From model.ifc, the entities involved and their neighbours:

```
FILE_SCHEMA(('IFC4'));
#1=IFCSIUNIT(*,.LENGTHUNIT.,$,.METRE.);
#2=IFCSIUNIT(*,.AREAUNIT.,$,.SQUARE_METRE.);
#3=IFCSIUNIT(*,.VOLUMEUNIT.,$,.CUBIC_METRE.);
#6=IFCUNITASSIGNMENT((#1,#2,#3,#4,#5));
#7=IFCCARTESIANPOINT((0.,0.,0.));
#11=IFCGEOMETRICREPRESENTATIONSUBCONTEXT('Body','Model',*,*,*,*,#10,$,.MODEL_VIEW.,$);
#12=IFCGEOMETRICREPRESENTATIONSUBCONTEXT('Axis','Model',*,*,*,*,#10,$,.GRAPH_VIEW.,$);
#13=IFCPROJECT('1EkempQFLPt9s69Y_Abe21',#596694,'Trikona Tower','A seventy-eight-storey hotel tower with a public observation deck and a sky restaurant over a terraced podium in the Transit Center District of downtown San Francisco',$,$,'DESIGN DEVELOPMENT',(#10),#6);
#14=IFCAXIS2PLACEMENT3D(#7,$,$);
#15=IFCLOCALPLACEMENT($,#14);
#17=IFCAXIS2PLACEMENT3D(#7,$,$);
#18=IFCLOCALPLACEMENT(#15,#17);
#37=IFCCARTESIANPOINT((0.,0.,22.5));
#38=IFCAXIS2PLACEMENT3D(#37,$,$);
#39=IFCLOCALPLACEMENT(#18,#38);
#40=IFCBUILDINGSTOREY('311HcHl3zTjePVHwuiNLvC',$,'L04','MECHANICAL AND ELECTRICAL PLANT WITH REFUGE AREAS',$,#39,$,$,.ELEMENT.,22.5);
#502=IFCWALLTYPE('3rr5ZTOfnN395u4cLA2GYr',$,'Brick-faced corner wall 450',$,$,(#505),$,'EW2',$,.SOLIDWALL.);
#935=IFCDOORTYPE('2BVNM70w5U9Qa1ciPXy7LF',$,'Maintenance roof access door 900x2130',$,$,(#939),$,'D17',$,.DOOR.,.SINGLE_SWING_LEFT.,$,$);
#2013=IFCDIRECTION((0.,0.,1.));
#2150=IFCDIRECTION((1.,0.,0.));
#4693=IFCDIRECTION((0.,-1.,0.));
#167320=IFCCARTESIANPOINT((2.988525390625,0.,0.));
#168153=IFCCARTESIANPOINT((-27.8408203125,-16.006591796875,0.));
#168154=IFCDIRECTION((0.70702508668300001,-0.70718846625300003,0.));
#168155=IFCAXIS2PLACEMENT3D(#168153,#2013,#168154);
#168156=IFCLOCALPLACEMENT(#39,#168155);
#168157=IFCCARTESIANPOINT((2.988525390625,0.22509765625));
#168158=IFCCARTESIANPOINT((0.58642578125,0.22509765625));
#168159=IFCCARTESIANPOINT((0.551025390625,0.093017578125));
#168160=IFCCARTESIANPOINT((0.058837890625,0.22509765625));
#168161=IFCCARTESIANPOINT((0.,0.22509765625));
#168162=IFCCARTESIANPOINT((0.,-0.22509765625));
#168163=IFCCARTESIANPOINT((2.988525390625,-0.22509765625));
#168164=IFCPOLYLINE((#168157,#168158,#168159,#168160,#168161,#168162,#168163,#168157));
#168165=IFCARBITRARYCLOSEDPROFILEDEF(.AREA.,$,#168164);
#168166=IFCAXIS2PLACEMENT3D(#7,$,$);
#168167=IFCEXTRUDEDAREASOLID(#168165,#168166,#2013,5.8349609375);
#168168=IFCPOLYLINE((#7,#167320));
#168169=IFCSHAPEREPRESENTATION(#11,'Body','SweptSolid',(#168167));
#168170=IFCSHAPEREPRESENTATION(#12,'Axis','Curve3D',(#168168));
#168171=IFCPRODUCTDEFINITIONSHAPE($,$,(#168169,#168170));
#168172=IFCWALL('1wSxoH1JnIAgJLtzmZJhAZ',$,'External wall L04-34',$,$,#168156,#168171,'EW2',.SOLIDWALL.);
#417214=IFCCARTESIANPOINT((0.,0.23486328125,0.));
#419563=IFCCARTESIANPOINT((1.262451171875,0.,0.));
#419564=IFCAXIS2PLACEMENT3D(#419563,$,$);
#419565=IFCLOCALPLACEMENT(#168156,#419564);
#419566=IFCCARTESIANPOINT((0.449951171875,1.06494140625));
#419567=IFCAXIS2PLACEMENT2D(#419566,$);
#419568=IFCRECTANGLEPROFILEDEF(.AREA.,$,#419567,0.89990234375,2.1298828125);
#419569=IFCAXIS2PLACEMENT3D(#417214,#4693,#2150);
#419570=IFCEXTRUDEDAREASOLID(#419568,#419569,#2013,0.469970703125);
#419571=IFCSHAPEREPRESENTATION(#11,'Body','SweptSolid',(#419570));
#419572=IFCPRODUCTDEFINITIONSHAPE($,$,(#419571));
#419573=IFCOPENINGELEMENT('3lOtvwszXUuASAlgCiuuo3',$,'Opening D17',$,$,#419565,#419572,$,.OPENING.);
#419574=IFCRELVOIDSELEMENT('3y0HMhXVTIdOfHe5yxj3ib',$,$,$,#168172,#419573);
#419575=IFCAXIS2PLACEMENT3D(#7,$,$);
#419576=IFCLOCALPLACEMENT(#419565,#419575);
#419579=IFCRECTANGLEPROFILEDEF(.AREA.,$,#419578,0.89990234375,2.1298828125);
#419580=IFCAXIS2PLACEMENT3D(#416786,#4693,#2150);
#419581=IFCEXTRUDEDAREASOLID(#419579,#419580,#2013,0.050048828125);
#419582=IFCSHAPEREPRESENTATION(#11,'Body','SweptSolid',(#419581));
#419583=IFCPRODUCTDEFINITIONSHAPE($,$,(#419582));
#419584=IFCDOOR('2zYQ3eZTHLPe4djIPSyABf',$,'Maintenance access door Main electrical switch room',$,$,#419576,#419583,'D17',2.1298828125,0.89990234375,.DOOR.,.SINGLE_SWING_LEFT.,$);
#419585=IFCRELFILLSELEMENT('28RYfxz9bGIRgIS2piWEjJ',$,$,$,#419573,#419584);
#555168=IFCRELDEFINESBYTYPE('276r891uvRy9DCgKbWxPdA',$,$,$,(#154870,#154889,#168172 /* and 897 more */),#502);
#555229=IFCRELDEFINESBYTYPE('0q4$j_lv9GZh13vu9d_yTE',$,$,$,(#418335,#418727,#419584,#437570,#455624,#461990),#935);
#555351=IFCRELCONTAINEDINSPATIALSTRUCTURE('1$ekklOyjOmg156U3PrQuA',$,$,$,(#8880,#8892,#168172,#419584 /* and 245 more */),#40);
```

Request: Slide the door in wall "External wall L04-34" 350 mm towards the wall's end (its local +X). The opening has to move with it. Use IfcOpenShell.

```python
import ifcopenshell
import ifcopenshell.api.geometry
import ifcopenshell.util.placement
import ifcopenshell.util.unit

model = ifcopenshell.open("model.ifc")
unit_scale = ifcopenshell.util.unit.calculate_unit_scale(model)

door = model.by_guid("2zYQ3eZTHLPe4djIPSyABf")
opening = door.FillsVoids[0].RelatingOpeningElement
wall = opening.VoidsElements[0].RelatingBuildingElement

wall_matrix = ifcopenshell.util.placement.get_local_placement(wall.ObjectPlacement)
shift = wall_matrix[:3, 0] * 0.35 / unit_scale
before = ifcopenshell.util.placement.get_local_placement(door.ObjectPlacement)[:3, 3].copy()

# The door is placed relative to its opening, so it follows when the opening moves.
matrix = ifcopenshell.util.placement.get_local_placement(opening.ObjectPlacement)
matrix[:3, 3] += shift
ifcopenshell.api.geometry.edit_object_placement(
    model, product=opening, matrix=matrix, is_si=False, should_transform_children=True
)

after = ifcopenshell.util.placement.get_local_placement(door.ObjectPlacement)[:3, 3]
print("door moved by", (after - before).round(3) + 0.0)

model.write("model_updated.ifc")
```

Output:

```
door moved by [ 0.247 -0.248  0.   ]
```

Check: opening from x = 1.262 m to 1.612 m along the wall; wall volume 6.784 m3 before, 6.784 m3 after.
